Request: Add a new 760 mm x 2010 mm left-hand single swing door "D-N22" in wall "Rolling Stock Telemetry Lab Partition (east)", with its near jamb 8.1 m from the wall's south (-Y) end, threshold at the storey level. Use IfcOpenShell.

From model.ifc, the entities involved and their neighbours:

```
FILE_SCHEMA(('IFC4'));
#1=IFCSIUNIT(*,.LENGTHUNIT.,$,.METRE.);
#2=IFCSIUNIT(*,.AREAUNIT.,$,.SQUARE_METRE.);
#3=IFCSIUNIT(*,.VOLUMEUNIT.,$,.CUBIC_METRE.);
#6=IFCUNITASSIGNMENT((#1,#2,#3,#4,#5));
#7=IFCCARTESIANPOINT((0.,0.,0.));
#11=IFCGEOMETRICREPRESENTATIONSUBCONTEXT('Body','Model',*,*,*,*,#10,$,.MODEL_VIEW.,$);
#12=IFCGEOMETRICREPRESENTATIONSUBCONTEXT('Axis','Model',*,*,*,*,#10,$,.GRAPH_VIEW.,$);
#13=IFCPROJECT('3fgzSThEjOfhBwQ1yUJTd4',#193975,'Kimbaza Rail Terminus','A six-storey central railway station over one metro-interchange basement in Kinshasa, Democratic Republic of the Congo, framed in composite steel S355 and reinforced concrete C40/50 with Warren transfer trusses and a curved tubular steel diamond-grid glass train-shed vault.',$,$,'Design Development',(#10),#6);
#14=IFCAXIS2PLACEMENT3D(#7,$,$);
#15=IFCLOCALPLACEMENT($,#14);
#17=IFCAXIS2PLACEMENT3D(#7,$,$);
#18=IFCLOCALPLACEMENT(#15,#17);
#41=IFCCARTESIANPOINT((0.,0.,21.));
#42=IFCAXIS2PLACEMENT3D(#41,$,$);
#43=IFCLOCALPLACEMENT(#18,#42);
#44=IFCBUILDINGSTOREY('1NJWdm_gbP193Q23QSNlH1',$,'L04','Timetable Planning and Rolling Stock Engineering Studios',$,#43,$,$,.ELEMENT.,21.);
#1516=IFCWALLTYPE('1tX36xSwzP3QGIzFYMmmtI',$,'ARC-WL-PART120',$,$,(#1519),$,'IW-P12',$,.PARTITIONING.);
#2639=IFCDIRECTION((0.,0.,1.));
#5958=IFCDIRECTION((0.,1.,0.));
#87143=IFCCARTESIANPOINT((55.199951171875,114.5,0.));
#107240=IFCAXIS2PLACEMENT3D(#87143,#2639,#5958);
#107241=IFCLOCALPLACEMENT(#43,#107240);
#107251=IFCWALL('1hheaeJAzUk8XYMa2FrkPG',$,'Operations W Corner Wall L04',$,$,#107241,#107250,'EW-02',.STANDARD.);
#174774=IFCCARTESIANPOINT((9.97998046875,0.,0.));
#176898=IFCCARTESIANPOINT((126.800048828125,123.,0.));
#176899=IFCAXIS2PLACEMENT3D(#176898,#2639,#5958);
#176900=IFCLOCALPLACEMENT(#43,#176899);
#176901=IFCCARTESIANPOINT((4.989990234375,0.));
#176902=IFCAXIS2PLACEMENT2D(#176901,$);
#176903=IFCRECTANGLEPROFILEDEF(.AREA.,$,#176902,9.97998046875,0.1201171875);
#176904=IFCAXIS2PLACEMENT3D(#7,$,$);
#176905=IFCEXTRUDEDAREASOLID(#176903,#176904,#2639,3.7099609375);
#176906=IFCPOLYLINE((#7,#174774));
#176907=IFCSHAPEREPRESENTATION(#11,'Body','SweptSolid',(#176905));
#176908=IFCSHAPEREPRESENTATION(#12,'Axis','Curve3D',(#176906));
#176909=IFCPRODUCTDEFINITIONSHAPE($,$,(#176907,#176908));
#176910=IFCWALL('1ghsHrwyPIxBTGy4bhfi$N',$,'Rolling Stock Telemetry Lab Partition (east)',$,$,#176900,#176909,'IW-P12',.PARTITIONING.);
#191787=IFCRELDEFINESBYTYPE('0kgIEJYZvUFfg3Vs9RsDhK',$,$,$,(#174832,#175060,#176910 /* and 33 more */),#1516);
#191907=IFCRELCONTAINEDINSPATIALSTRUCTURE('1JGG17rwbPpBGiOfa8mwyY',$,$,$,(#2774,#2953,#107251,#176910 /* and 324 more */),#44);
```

```python
import numpy as np
import ifcopenshell
import ifcopenshell.api.feature
import ifcopenshell.api.geometry
import ifcopenshell.api.root
import ifcopenshell.api.spatial
import ifcopenshell.geom
import ifcopenshell.util.element
import ifcopenshell.util.placement
import ifcopenshell.util.representation
import ifcopenshell.util.shape
import ifcopenshell.util.unit

model = ifcopenshell.open("model.ifc")
unit_scale = ifcopenshell.util.unit.calculate_unit_scale(model)
settings = ifcopenshell.geom.settings()


def volume(element):
    """Net volume in cubic metres, openings subtracted."""
    shape = ifcopenshell.geom.create_shape(settings, element)
    return ifcopenshell.util.shape.get_volume(shape.geometry)


wall = model.by_id(176910)
storey = ifcopenshell.util.element.get_container(wall, ifc_class="IfcBuildingStorey")
context = ifcopenshell.util.representation.get_context(model, "Model", "Body", "MODEL_VIEW")
before = volume(wall)

width, height, from_end, sill = 0.76, 2.01, 8.1, 0.0  # metres

# The wall runs along its own X axis, and the end named is its -X end.
wall_shape = ifcopenshell.geom.create_shape(settings, wall)
x, y, z = ifcopenshell.util.shape.get_vertices(wall_shape.geometry).T
start = x.min() + from_end
face, thickness = float(y.min()), float(y.max() - y.min())
wall_matrix = ifcopenshell.util.placement.get_local_placement(wall.ObjectPlacement)
level = ifcopenshell.util.placement.get_local_placement(storey.ObjectPlacement)[2, 3]


def in_wall(x, y):
    """Placement at x, y metres in the wall's axes, at sill height."""
    matrix = wall_matrix.copy()
    matrix[:, 3] = wall_matrix @ np.array([x / unit_scale, y / unit_scale, 0.0, 1.0])
    matrix[2, 3] = level + sill / unit_scale
    return matrix


# Opening: a box that overshoots both wall faces by 50 mm.
opening = ifcopenshell.api.root.create_entity(model, ifc_class="IfcOpeningElement", predefined_type="OPENING")
box = ifcopenshell.api.geometry.add_wall_representation(
    model, context=context, length=width, height=height, thickness=thickness + 0.1
)
ifcopenshell.api.geometry.assign_representation(model, product=opening, representation=box)
ifcopenshell.api.geometry.edit_object_placement(model, product=opening, matrix=in_wall(start, face - 0.05), is_si=False)
ifcopenshell.api.feature.add_feature(model, feature=opening, element=wall)

door = ifcopenshell.api.root.create_entity(model, ifc_class="IfcDoor", name="D-N22", predefined_type="DOOR")
door.OverallWidth, door.OverallHeight = width / unit_scale, height / unit_scale
door.OperationType = "SINGLE_SWING_LEFT"
body = ifcopenshell.api.geometry.add_door_representation(
    model,
    context=context,
    overall_width=door.OverallWidth,
    overall_height=door.OverallHeight,
    operation_type="SINGLE_SWING_LEFT",
    lining_properties={"LiningDepth": thickness / unit_scale, "ThresholdDepth": thickness / unit_scale},
)
ifcopenshell.api.geometry.assign_representation(model, product=door, representation=body)
ifcopenshell.api.spatial.assign_container(model, products=[door], relating_structure=storey)
ifcopenshell.api.feature.add_filling(model, opening=opening, element=door)

# The lining spans the wall, so the door starts at the wall face.
ifcopenshell.api.geometry.edit_object_placement(model, product=door, matrix=in_wall(start, face), is_si=False)

after = volume(wall)

print(f"wall volume {before:.3f} -> {after:.3f} m3")

model.write("model_updated.ifc")
```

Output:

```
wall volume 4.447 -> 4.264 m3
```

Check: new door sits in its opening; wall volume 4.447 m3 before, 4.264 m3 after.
